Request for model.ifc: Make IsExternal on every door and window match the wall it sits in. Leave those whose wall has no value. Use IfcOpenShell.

First a look at what the model holds.

```python
import ifcopenshell
import ifcopenshell.util.element

model = ifcopenshell.open("model.ifc")
print(model.schema)
seen = {}
for e in model.by_type("IfcDoor") + model.by_type("IfcWindow"):
    if not e.FillsVoids:
        continue
    host = e.FillsVoids[0].RelatingOpeningElement.VoidsElements[0].RelatingBuildingElement
    own = ifcopenshell.util.element.get_pset(e, f"Pset_{e.is_a()[3:].removesuffix('StandardCase')}Common", "IsExternal")
    wall = ifcopenshell.util.element.get_pset(host, "Pset_WallCommon", "IsExternal")
    seen[e.is_a(), own, wall] = seen.get((e.is_a(), own, wall), 0) + 1
for (cls, own, wall), count in sorted(seen.items(), key=str):
    print(count, cls, "IsExternal:", own, "| host wall:", wall)
```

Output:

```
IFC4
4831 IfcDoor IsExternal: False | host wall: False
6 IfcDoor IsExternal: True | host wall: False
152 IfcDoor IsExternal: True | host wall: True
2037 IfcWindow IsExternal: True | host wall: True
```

```python
import ifcopenshell
import ifcopenshell.api.pset
import ifcopenshell.util.element

model = ifcopenshell.open("model.ifc")

count = 0
for ifc_class, pset_name in (("IfcDoor", "Pset_DoorCommon"), ("IfcWindow", "Pset_WindowCommon")):
    for e in model.by_type(ifc_class):
        if not e.FillsVoids:
            continue
        host = e.FillsVoids[0].RelatingOpeningElement.VoidsElements[0].RelatingBuildingElement
        external = ifcopenshell.util.element.get_pset(host, "Pset_WallCommon", "IsExternal")
        if external is None or ifcopenshell.util.element.get_pset(e, pset_name, "IsExternal") == external:
            continue
        pset = ifcopenshell.api.pset.add_pset(model, product=e, name=pset_name)
        ifcopenshell.api.pset.edit_pset(model, pset=pset, properties={"IsExternal": external})
        count += 1

print(count, "updated")

model.write("model-out.ifc")
```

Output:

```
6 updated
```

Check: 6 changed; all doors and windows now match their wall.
